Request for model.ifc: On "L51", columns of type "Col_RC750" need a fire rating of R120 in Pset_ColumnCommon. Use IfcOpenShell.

First a look at what the model holds.

```python
import ifcopenshell
import ifcopenshell.util.element

model = ifcopenshell.open("model.ifc")
print(model.schema)
storey = next(s for s in model.by_type("IfcBuildingStorey") if s.Name == "L51")
columns = [e for e in ifcopenshell.util.element.get_decomposition(storey) if e.is_a("IfcColumn")]
seen = {}
for e in columns:
    element_type = ifcopenshell.util.element.get_type(e)
    key = (element_type.Name if element_type != e and element_type else None, ifcopenshell.util.element.get_pset(e, "Pset_ColumnCommon", "FireRating"))
    seen[key] = seen.get(key, 0) + 1
for (name, value), count in sorted(seen.items(), key=str):
    print(count, "x", name, "|", value)
```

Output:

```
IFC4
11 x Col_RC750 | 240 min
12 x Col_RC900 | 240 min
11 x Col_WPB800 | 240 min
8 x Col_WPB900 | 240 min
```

```python
import ifcopenshell
import ifcopenshell.api.pset
import ifcopenshell.util.element

model = ifcopenshell.open("model.ifc")

storey = next(s for s in model.by_type("IfcBuildingStorey") if s.Name == "L51")
columns = [e for e in ifcopenshell.util.element.get_decomposition(storey) if e.is_a("IfcColumn")]

count = 0
for e in columns:
    element_type = ifcopenshell.util.element.get_type(e)
    if element_type in (None, e) or element_type.Name != "Col_RC750":
        continue
    found = ifcopenshell.util.element.get_pset(e, "Pset_ColumnCommon", should_inherit=False)
    if found:
        pset = model.by_id(found["id"])
        if len(ifcopenshell.util.element.get_elements_by_pset(pset)) > 1:
            pset = ifcopenshell.api.pset.unshare_pset(model, products=[e], pset=pset)[0]
    else:
        pset = ifcopenshell.api.pset.add_pset(model, product=e, name="Pset_ColumnCommon")
    ifcopenshell.api.pset.edit_pset(model, pset=pset, properties={"FireRating": "R120"})
    count += 1

print(count, "columns updated")

model.write("model_v2.ifc")
```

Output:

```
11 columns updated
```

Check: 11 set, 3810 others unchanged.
